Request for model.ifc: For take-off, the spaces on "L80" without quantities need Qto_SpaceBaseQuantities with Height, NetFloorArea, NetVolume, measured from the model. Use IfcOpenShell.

First a look at what the model holds.

```python
import ifcopenshell
import ifcopenshell.util.element
import ifcopenshell.util.unit

model = ifcopenshell.open("model.ifc")
print(model.schema)
for unit_type in ("LENGTHUNIT", "AREAUNIT", "VOLUMEUNIT"):
    print(unit_type, ifcopenshell.util.unit.calculate_unit_scale(model, unit_type))
storey = next(s for s in model.by_type("IfcBuildingStorey") if s.Name == "L80")
spaces = [e for e in ifcopenshell.util.element.get_decomposition(storey) if e.is_a("IfcSpace")]
for e in sorted(spaces, key=lambda e: e.id()):
    print(e.id(), e.is_a(), e.Name, list(ifcopenshell.util.element.get_psets(e, qtos_only=True)), sep=" | ")
```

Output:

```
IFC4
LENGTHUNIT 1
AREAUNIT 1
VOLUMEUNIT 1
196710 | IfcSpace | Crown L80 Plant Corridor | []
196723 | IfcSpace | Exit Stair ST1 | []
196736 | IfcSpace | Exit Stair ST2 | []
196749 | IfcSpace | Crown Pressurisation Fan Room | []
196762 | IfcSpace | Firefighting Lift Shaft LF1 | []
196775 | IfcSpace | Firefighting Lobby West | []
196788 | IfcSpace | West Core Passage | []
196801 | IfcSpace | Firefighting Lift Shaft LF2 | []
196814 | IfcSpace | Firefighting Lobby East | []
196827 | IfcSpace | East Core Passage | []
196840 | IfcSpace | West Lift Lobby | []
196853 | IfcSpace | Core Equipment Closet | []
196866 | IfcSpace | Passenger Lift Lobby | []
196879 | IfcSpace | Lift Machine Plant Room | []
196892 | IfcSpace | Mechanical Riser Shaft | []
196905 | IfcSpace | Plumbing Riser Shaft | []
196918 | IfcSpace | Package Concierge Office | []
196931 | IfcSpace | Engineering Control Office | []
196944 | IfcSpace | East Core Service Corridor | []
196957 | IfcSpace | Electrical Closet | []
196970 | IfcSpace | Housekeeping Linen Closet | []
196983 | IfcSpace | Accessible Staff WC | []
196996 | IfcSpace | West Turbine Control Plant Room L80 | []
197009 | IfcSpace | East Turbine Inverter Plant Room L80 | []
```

```python
import ifcopenshell
import ifcopenshell.api.pset
import ifcopenshell.geom
import ifcopenshell.util.element
import ifcopenshell.util.shape
import ifcopenshell.util.unit

model = ifcopenshell.open("model.ifc")
unit_scale = ifcopenshell.util.unit.calculate_unit_scale(model)
area_scale = ifcopenshell.util.unit.calculate_unit_scale(model, "AREAUNIT")
volume_scale = ifcopenshell.util.unit.calculate_unit_scale(model, "VOLUMEUNIT")
settings = ifcopenshell.geom.settings()

storey = next(s for s in model.by_type("IfcBuildingStorey") if s.Name == "L80")
spaces = [e for e in ifcopenshell.util.element.get_decomposition(storey) if e.is_a("IfcSpace")]

for e in sorted(spaces, key=lambda e: e.id()):
    if ifcopenshell.util.element.get_psets(e, qtos_only=True, should_inherit=False):
        continue
    # Geometry comes back in metres, in the element's own axes.
    shape = ifcopenshell.geom.create_shape(settings, e)
    values = {
        "Height": ifcopenshell.util.shape.get_z(shape.geometry) / unit_scale,
        "NetFloorArea": ifcopenshell.util.shape.get_footprint_area(shape.geometry) / area_scale,
        "NetVolume": ifcopenshell.util.shape.get_volume(shape.geometry) / volume_scale,
    }
    qto = ifcopenshell.api.pset.add_qto(model, product=e, name="Qto_SpaceBaseQuantities")
    ifcopenshell.api.pset.edit_qto(model, qto=qto, properties=values)
    print(e.id(), {k: round(v, 3) for k, v in values.items()})

model.write("model_v2.ifc")
```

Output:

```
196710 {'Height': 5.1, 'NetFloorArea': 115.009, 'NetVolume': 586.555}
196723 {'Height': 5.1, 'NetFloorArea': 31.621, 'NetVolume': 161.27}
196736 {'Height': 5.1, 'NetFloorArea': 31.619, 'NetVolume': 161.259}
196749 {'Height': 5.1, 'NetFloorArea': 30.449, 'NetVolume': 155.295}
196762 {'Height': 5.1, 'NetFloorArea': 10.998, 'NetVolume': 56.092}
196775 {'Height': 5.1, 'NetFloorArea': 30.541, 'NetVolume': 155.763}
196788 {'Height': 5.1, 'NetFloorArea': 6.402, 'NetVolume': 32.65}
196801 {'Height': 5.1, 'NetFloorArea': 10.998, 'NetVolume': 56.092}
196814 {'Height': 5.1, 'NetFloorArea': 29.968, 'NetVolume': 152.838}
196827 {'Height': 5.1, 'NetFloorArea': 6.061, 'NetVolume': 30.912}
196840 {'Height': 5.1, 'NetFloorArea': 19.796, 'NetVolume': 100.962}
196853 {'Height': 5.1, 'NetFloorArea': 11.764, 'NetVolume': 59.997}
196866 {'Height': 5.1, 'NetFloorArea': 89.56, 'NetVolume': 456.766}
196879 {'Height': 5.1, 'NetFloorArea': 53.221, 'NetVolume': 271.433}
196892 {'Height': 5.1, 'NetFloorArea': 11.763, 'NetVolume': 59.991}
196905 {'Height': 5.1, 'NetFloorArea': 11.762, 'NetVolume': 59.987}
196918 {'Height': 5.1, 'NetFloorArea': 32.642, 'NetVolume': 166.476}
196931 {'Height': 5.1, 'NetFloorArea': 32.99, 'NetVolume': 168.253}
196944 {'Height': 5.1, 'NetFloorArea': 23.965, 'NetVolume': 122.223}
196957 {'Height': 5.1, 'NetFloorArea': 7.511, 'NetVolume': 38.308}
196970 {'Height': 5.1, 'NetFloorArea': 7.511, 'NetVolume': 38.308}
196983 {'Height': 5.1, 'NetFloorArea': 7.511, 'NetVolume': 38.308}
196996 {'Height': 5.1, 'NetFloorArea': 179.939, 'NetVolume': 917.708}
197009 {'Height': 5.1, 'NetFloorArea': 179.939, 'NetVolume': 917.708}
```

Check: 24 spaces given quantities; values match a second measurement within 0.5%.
